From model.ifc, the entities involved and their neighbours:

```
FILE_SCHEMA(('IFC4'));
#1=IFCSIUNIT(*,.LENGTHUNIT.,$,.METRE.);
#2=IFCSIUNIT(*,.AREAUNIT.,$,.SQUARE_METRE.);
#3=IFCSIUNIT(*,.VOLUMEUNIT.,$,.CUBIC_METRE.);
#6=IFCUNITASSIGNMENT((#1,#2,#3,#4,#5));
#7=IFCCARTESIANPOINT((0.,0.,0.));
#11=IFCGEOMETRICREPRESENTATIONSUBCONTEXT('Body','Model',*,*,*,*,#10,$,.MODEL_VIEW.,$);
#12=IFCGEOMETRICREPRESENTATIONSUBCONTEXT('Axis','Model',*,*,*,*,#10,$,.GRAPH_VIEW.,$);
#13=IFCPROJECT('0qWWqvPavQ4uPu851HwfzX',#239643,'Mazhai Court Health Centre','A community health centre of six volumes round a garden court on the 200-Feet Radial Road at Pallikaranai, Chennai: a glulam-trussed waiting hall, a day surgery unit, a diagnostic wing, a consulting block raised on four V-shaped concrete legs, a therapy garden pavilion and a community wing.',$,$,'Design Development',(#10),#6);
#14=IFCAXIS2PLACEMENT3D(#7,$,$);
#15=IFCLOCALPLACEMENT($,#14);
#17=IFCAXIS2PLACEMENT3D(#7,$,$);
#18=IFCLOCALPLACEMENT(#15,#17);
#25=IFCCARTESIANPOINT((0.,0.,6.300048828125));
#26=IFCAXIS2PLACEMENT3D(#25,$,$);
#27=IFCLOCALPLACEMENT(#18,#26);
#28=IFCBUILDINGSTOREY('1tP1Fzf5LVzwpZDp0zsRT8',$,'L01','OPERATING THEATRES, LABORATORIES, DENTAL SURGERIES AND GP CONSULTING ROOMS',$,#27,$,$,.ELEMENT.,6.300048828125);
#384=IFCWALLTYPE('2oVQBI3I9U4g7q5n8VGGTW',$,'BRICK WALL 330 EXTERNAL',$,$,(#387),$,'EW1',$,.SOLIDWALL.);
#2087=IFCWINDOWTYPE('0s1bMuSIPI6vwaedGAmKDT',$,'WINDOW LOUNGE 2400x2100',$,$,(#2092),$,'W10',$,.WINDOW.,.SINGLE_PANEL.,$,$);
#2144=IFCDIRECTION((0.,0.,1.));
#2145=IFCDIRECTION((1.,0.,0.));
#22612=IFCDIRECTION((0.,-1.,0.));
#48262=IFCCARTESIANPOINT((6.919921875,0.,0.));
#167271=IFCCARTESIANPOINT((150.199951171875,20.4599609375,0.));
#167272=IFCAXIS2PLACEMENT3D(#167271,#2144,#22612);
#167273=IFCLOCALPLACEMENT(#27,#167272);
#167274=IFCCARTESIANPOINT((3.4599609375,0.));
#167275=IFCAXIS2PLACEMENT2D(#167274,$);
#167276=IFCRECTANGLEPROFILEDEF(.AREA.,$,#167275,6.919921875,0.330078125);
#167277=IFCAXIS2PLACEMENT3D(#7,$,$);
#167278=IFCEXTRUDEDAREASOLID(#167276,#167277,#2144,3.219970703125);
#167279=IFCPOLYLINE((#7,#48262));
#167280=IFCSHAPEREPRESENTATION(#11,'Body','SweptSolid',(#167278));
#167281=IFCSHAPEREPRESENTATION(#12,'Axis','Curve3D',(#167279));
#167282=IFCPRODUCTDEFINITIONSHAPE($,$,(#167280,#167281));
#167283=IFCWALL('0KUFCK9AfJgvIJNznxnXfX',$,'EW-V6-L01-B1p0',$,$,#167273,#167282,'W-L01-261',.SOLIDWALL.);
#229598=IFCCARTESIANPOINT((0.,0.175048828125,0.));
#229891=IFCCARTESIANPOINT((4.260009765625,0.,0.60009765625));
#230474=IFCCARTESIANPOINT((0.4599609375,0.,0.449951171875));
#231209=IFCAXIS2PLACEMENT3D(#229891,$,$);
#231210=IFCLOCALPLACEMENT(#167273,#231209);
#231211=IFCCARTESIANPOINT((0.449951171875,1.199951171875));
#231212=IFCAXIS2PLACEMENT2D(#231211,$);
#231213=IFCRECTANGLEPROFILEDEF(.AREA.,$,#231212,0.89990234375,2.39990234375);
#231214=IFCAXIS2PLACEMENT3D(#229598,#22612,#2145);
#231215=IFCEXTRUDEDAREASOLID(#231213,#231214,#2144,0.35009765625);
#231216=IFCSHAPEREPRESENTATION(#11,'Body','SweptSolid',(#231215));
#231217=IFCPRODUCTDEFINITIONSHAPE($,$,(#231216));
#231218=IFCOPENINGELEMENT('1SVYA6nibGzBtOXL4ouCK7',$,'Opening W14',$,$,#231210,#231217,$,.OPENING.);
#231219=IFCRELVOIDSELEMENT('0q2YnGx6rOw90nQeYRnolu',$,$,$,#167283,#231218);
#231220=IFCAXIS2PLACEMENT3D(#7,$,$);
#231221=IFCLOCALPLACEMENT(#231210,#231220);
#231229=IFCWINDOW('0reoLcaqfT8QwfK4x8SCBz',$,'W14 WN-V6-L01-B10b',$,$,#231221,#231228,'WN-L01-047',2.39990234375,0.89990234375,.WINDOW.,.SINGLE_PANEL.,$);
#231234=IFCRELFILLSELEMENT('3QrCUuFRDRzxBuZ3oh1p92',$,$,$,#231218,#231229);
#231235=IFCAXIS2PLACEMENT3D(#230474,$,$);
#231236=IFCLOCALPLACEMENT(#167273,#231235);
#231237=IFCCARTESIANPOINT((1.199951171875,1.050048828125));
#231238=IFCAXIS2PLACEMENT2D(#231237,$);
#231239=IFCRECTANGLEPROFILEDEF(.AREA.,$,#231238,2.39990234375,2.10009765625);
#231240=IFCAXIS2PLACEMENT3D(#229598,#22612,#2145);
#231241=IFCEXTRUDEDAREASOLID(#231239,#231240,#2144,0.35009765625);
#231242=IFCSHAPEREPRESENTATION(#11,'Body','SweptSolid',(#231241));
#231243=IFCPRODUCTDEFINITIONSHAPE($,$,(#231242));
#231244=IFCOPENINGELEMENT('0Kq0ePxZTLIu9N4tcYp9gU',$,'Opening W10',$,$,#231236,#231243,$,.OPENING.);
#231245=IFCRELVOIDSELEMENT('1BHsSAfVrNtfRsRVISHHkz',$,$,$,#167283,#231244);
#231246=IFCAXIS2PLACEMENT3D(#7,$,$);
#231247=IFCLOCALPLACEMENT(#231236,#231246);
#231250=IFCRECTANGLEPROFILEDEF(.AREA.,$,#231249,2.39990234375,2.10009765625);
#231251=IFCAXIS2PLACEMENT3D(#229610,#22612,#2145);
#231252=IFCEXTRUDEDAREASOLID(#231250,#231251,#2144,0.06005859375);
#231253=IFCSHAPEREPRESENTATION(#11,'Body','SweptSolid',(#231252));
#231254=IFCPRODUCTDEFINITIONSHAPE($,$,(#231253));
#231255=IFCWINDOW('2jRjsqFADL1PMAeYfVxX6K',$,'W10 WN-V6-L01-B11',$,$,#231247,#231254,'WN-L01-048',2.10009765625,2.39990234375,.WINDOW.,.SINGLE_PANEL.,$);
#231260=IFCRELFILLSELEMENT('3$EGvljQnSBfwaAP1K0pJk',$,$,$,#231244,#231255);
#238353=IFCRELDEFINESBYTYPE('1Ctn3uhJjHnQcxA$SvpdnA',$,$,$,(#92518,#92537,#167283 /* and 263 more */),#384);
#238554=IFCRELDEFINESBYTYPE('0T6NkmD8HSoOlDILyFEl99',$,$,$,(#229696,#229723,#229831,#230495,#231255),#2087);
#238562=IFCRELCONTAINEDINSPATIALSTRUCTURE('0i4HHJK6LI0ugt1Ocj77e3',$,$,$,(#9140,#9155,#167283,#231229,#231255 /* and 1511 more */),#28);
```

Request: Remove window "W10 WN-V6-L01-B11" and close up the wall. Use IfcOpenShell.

```python
import ifcopenshell
import ifcopenshell.api.feature
import ifcopenshell.api.root
import ifcopenshell.geom
import ifcopenshell.util.shape

model = ifcopenshell.open("model.ifc")
settings = ifcopenshell.geom.settings()


def volume(element):
    """Net volume in cubic metres, openings subtracted."""
    shape = ifcopenshell.geom.create_shape(settings, element)
    return ifcopenshell.util.shape.get_volume(shape.geometry)


window = model.by_guid("2jRjsqFADL1PMAeYfVxX6K")
opening = window.FillsVoids[0].RelatingOpeningElement
wall = opening.VoidsElements[0].RelatingBuildingElement
before = volume(wall)

ifcopenshell.api.root.remove_product(model, product=window)
ifcopenshell.api.feature.remove_feature(model, feature=opening)

after = volume(wall)

print(f"wall volume {before:.3f} -> {after:.3f} m3")

model.write("model_rev.ifc")
```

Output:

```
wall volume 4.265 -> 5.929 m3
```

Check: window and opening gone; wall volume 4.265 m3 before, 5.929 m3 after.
